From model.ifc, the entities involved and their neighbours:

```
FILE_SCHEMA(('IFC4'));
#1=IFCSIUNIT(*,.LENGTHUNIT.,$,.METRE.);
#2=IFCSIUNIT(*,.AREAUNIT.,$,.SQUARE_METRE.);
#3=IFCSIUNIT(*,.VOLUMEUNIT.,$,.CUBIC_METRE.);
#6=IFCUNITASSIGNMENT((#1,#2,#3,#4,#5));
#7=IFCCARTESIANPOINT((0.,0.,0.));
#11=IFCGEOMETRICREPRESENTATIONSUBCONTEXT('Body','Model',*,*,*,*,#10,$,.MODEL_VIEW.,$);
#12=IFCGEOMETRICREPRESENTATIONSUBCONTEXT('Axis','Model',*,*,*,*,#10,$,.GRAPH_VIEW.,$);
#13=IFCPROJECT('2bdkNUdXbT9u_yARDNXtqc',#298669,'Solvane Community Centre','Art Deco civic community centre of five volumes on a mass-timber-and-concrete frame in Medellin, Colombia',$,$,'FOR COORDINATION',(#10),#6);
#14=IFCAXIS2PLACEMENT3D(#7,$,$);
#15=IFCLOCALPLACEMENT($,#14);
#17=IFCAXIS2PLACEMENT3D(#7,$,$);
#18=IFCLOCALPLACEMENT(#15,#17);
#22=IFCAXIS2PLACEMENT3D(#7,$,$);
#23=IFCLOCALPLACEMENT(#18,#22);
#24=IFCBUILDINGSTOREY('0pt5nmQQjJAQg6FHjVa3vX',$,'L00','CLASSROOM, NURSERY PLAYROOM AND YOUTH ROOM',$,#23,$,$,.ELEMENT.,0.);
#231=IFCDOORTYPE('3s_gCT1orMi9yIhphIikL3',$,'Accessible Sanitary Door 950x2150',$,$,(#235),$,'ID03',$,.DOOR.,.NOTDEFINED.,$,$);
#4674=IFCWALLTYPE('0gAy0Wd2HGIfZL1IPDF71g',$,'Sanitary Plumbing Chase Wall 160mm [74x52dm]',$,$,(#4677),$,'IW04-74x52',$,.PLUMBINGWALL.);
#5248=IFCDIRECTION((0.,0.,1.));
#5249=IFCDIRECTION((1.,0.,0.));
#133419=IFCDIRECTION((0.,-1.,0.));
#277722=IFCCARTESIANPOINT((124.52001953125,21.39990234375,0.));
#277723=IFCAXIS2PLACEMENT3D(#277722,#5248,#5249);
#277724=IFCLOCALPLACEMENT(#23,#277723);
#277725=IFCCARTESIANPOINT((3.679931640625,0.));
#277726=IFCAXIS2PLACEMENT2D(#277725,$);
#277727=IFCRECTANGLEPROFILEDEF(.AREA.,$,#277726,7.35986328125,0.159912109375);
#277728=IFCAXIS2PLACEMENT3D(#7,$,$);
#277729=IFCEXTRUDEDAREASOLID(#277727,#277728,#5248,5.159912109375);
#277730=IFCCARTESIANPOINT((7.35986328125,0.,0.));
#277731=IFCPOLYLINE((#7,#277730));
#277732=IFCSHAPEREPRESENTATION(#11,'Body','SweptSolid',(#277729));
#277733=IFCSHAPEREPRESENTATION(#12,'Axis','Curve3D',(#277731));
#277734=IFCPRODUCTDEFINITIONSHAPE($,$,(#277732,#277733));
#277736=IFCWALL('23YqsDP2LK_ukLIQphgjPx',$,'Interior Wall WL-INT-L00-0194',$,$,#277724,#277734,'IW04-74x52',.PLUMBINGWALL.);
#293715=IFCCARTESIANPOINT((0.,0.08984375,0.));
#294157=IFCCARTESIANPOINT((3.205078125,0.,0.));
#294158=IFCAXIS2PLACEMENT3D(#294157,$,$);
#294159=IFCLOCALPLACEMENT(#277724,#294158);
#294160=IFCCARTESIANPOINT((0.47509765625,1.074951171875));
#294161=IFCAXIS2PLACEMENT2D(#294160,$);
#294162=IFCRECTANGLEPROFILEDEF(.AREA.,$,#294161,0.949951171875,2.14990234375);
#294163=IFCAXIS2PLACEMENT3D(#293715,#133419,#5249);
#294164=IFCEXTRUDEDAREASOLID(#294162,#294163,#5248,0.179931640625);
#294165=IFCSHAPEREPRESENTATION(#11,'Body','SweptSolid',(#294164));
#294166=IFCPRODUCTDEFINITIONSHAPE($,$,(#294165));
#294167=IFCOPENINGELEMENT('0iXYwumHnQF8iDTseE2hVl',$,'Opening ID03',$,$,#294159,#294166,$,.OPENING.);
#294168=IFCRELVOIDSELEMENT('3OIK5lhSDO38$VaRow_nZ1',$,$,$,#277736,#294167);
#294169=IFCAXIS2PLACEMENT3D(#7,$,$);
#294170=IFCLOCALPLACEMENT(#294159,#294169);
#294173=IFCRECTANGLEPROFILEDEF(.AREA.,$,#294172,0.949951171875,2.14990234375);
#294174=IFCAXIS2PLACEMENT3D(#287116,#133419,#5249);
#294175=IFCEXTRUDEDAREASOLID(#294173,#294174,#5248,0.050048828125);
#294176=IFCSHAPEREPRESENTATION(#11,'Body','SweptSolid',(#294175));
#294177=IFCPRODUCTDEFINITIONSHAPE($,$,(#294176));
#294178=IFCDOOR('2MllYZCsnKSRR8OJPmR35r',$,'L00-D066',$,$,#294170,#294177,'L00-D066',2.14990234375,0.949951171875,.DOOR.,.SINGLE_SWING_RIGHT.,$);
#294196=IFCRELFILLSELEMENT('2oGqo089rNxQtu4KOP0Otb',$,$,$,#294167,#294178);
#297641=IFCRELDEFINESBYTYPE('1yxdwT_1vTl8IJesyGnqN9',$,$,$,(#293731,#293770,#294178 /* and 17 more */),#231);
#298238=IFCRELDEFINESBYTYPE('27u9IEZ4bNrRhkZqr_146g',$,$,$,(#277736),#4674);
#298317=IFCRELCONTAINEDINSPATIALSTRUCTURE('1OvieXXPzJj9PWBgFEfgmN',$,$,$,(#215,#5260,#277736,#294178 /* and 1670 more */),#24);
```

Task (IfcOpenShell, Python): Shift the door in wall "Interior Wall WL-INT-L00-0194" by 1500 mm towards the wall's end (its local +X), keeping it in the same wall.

```python
import ifcopenshell
import ifcopenshell.api.geometry
import ifcopenshell.util.placement

model = ifcopenshell.open("model.ifc")

door = model.by_guid("2MllYZCsnKSRR8OJPmR35r")
opening = door.FillsVoids[0].RelatingOpeningElement
wall = opening.VoidsElements[0].RelatingBuildingElement

wall_matrix = ifcopenshell.util.placement.get_local_placement(wall.ObjectPlacement)
shift = wall_matrix[:3, 0] * 1.5
before = ifcopenshell.util.placement.get_local_placement(door.ObjectPlacement)[:3, 3].copy()

# The door is placed relative to its opening, so it follows when the opening moves.
matrix = ifcopenshell.util.placement.get_local_placement(opening.ObjectPlacement)
matrix[:3, 3] += shift
ifcopenshell.api.geometry.edit_object_placement(
    model, product=opening, matrix=matrix, is_si=False, should_transform_children=True
)

after = ifcopenshell.util.placement.get_local_placement(door.ObjectPlacement)[:3, 3]
print("door moved by", (after - before).round(3) + 0.0)

model.write("model_v2.ifc")
```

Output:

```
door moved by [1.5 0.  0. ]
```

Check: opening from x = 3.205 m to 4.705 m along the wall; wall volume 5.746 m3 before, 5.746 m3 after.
